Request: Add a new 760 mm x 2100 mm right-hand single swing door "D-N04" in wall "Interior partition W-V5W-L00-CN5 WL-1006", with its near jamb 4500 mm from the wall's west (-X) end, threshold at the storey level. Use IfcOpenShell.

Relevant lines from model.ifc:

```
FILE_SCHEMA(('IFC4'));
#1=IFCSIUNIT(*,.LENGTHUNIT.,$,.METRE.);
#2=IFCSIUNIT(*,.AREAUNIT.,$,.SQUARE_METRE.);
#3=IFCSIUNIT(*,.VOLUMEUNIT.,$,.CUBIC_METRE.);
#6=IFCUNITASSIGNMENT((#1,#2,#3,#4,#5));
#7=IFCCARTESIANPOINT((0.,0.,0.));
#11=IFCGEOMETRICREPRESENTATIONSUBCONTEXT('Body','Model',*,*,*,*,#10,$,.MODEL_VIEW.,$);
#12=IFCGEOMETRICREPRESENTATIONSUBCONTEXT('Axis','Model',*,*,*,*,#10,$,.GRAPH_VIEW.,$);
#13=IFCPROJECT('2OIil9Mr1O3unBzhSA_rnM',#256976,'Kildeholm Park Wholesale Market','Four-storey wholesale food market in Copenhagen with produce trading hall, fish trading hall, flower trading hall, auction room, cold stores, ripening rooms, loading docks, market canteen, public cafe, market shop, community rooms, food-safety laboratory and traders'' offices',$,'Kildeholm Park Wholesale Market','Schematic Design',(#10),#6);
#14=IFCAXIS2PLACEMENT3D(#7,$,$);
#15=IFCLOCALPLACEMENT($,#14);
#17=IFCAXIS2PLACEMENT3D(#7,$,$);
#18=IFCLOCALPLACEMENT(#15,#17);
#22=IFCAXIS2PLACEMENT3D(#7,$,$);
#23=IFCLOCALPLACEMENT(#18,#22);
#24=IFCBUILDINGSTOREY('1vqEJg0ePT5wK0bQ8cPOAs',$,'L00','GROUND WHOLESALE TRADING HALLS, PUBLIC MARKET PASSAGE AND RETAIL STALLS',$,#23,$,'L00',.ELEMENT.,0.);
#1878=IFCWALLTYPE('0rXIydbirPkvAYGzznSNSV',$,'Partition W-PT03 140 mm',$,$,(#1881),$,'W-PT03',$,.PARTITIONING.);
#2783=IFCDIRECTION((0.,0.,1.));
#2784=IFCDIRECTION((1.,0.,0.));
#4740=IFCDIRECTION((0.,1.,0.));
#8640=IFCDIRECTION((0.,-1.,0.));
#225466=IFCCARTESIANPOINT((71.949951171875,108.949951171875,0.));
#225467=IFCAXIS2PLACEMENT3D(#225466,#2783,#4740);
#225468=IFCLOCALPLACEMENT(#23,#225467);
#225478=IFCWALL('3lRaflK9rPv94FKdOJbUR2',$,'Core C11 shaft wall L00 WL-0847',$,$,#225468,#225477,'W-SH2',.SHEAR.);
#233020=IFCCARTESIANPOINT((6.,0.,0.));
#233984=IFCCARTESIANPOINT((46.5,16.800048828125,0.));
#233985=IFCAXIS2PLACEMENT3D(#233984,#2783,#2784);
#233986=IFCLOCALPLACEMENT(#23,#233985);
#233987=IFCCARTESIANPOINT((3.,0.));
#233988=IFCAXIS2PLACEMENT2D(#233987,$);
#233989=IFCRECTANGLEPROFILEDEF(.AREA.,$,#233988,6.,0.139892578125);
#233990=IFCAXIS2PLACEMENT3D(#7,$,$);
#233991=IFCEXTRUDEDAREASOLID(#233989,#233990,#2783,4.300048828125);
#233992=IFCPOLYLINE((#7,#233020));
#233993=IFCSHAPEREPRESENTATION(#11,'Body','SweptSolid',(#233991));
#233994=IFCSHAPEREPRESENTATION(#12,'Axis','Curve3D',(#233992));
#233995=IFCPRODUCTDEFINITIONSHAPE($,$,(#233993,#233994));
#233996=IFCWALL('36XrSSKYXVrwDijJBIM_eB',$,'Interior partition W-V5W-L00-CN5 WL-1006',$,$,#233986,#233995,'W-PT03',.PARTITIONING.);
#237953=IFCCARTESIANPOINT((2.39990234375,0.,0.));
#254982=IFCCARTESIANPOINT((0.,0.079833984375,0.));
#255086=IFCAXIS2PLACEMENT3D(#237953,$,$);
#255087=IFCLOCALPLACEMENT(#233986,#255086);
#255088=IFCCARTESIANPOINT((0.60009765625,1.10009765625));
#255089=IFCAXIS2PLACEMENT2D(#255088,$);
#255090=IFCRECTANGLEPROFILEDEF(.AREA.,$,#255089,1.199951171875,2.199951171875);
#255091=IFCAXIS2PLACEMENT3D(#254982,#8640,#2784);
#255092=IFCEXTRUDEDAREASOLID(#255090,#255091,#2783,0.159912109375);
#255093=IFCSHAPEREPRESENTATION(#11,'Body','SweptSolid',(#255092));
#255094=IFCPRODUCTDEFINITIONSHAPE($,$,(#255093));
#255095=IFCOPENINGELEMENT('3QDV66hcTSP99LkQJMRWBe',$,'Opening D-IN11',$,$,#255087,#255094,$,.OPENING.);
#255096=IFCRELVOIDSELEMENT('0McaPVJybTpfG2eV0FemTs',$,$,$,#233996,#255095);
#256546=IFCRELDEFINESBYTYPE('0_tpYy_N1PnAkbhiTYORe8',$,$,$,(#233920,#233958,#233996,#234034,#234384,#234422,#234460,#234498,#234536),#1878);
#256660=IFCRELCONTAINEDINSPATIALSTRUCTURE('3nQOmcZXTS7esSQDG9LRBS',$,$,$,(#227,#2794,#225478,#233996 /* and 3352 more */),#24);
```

```python
import numpy as np
import ifcopenshell
import ifcopenshell.api.feature
import ifcopenshell.api.geometry
import ifcopenshell.api.root
import ifcopenshell.api.spatial
import ifcopenshell.geom
import ifcopenshell.util.element
import ifcopenshell.util.placement
import ifcopenshell.util.representation
import ifcopenshell.util.shape
import ifcopenshell.util.unit

model = ifcopenshell.open("model.ifc")
unit_scale = ifcopenshell.util.unit.calculate_unit_scale(model)
settings = ifcopenshell.geom.settings()


def volume(element):
    """Net volume in cubic metres, openings subtracted."""
    shape = ifcopenshell.geom.create_shape(settings, element)
    return ifcopenshell.util.shape.get_volume(shape.geometry)


wall = model.by_id(233996)
storey = ifcopenshell.util.element.get_container(wall, ifc_class="IfcBuildingStorey")
context = ifcopenshell.util.representation.get_context(model, "Model", "Body", "MODEL_VIEW")
before = volume(wall)

width, height, from_end, sill = 0.76, 2.1, 4.5, 0.0  # metres

# The wall runs along its own X axis, and the end named is its -X end.
wall_shape = ifcopenshell.geom.create_shape(settings, wall)
x, y, z = ifcopenshell.util.shape.get_vertices(wall_shape.geometry).T
start = x.min() + from_end
face, thickness = float(y.min()), float(y.max() - y.min())
wall_matrix = ifcopenshell.util.placement.get_local_placement(wall.ObjectPlacement)
level = ifcopenshell.util.placement.get_local_placement(storey.ObjectPlacement)[2, 3]


def in_wall(x, y):
    """Placement at x, y metres in the wall's axes, at sill height."""
    matrix = wall_matrix.copy()
    matrix[:, 3] = wall_matrix @ np.array([x / unit_scale, y / unit_scale, 0.0, 1.0])
    matrix[2, 3] = level + sill / unit_scale
    return matrix


# Opening: a box that overshoots both wall faces by 50 mm.
opening = ifcopenshell.api.root.create_entity(model, ifc_class="IfcOpeningElement", predefined_type="OPENING")
box = ifcopenshell.api.geometry.add_wall_representation(
    model, context=context, length=width, height=height, thickness=thickness + 0.1
)
ifcopenshell.api.geometry.assign_representation(model, product=opening, representation=box)
ifcopenshell.api.geometry.edit_object_placement(model, product=opening, matrix=in_wall(start, face - 0.05), is_si=False)
ifcopenshell.api.feature.add_feature(model, feature=opening, element=wall)

door = ifcopenshell.api.root.create_entity(model, ifc_class="IfcDoor", name="D-N04", predefined_type="DOOR")
door.OverallWidth, door.OverallHeight = width / unit_scale, height / unit_scale
door.OperationType = "SINGLE_SWING_RIGHT"
body = ifcopenshell.api.geometry.add_door_representation(
    model,
    context=context,
    overall_width=door.OverallWidth,
    overall_height=door.OverallHeight,
    operation_type="SINGLE_SWING_RIGHT",
    lining_properties={"LiningDepth": thickness / unit_scale, "ThresholdDepth": thickness / unit_scale},
)
ifcopenshell.api.geometry.assign_representation(model, product=door, representation=body)
ifcopenshell.api.spatial.assign_container(model, products=[door], relating_structure=storey)
ifcopenshell.api.feature.add_filling(model, opening=opening, element=door)

# The lining spans the wall, so the door starts at the wall face.
ifcopenshell.api.geometry.edit_object_placement(model, product=door, matrix=in_wall(start, face), is_si=False)

after = volume(wall)

print(f"wall volume {before:.3f} -> {after:.3f} m3")

model.write("model_updated.ifc")
```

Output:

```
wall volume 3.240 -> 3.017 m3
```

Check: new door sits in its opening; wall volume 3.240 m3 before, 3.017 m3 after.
